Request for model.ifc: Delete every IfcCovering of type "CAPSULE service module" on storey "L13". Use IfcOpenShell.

First a look at what the model holds.

```python
import ifcopenshell
import ifcopenshell.util.element

model = ifcopenshell.open("model.ifc")
print(model.schema)
storey = next(s for s in model.by_type("IfcBuildingStorey") if s.Name == "L13")
coverings = [e for e in ifcopenshell.util.element.get_decomposition(storey) if e.is_a("IfcCovering")]
seen = {}
for e in coverings:
    element_type = ifcopenshell.util.element.get_type(e)
    name = element_type.Name if element_type not in (None, e) else None
    seen[name] = seen.get(name, 0) + 1
for name, count in sorted(seen.items(), key=str):
    print(count, "x", name)
```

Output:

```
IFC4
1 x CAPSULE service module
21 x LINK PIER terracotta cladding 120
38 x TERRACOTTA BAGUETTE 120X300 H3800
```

```python
import ifcopenshell
import ifcopenshell.api.root
import ifcopenshell.util.element

model = ifcopenshell.open("model.ifc")

storey = next(s for s in model.by_type("IfcBuildingStorey") if s.Name == "L13")
coverings = [e for e in ifcopenshell.util.element.get_decomposition(storey) if e.is_a("IfcCovering")]
targets = [e for e in coverings if (t := ifcopenshell.util.element.get_type(e)) not in (None, e) and t.Name == "CAPSULE service module"]

for e in targets:
    ifcopenshell.api.root.remove_product(model, product=e)
print(len(targets), "removed")

model.write("model-out.ifc")
```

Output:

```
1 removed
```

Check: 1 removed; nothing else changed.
